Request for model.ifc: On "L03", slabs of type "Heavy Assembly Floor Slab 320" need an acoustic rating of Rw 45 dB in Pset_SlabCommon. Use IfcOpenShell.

First a look at what the model holds.

```python
import ifcopenshell
import ifcopenshell.util.element

model = ifcopenshell.open("model.ifc")
print(model.schema)
storey = next(s for s in model.by_type("IfcBuildingStorey") if s.Name == "L03")
slabs = [e for e in ifcopenshell.util.element.get_decomposition(storey) if e.is_a("IfcSlab")]
seen = {}
for e in slabs:
    element_type = ifcopenshell.util.element.get_type(e)
    key = (element_type.Name if element_type != e and element_type else None, ifcopenshell.util.element.get_pset(e, "Pset_SlabCommon", "AcousticRating"))
    seen[key] = seen.get(key, 0) + 1
for (name, value), count in sorted(seen.items(), key=str):
    print(count, "x", name, "|", value)
```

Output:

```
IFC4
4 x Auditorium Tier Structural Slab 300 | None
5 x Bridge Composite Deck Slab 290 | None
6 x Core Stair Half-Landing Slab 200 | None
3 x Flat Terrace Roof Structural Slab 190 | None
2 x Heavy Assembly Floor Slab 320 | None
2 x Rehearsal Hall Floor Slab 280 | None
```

```python
import ifcopenshell
import ifcopenshell.api.pset
import ifcopenshell.util.element

model = ifcopenshell.open("model.ifc")

storey = next(s for s in model.by_type("IfcBuildingStorey") if s.Name == "L03")
slabs = [e for e in ifcopenshell.util.element.get_decomposition(storey) if e.is_a("IfcSlab")]

count = 0
for e in slabs:
    element_type = ifcopenshell.util.element.get_type(e)
    if element_type in (None, e) or element_type.Name != "Heavy Assembly Floor Slab 320":
        continue
    # add_pset returns the element's existing set when there is one.
    pset = ifcopenshell.api.pset.add_pset(model, product=e, name="Pset_SlabCommon")
    ifcopenshell.api.pset.edit_pset(model, pset=pset, properties={"AcousticRating": "Rw 45 dB"})
    count += 1

print(count, "slabs updated")

model.write("model_updated.ifc")
```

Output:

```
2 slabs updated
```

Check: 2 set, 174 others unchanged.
